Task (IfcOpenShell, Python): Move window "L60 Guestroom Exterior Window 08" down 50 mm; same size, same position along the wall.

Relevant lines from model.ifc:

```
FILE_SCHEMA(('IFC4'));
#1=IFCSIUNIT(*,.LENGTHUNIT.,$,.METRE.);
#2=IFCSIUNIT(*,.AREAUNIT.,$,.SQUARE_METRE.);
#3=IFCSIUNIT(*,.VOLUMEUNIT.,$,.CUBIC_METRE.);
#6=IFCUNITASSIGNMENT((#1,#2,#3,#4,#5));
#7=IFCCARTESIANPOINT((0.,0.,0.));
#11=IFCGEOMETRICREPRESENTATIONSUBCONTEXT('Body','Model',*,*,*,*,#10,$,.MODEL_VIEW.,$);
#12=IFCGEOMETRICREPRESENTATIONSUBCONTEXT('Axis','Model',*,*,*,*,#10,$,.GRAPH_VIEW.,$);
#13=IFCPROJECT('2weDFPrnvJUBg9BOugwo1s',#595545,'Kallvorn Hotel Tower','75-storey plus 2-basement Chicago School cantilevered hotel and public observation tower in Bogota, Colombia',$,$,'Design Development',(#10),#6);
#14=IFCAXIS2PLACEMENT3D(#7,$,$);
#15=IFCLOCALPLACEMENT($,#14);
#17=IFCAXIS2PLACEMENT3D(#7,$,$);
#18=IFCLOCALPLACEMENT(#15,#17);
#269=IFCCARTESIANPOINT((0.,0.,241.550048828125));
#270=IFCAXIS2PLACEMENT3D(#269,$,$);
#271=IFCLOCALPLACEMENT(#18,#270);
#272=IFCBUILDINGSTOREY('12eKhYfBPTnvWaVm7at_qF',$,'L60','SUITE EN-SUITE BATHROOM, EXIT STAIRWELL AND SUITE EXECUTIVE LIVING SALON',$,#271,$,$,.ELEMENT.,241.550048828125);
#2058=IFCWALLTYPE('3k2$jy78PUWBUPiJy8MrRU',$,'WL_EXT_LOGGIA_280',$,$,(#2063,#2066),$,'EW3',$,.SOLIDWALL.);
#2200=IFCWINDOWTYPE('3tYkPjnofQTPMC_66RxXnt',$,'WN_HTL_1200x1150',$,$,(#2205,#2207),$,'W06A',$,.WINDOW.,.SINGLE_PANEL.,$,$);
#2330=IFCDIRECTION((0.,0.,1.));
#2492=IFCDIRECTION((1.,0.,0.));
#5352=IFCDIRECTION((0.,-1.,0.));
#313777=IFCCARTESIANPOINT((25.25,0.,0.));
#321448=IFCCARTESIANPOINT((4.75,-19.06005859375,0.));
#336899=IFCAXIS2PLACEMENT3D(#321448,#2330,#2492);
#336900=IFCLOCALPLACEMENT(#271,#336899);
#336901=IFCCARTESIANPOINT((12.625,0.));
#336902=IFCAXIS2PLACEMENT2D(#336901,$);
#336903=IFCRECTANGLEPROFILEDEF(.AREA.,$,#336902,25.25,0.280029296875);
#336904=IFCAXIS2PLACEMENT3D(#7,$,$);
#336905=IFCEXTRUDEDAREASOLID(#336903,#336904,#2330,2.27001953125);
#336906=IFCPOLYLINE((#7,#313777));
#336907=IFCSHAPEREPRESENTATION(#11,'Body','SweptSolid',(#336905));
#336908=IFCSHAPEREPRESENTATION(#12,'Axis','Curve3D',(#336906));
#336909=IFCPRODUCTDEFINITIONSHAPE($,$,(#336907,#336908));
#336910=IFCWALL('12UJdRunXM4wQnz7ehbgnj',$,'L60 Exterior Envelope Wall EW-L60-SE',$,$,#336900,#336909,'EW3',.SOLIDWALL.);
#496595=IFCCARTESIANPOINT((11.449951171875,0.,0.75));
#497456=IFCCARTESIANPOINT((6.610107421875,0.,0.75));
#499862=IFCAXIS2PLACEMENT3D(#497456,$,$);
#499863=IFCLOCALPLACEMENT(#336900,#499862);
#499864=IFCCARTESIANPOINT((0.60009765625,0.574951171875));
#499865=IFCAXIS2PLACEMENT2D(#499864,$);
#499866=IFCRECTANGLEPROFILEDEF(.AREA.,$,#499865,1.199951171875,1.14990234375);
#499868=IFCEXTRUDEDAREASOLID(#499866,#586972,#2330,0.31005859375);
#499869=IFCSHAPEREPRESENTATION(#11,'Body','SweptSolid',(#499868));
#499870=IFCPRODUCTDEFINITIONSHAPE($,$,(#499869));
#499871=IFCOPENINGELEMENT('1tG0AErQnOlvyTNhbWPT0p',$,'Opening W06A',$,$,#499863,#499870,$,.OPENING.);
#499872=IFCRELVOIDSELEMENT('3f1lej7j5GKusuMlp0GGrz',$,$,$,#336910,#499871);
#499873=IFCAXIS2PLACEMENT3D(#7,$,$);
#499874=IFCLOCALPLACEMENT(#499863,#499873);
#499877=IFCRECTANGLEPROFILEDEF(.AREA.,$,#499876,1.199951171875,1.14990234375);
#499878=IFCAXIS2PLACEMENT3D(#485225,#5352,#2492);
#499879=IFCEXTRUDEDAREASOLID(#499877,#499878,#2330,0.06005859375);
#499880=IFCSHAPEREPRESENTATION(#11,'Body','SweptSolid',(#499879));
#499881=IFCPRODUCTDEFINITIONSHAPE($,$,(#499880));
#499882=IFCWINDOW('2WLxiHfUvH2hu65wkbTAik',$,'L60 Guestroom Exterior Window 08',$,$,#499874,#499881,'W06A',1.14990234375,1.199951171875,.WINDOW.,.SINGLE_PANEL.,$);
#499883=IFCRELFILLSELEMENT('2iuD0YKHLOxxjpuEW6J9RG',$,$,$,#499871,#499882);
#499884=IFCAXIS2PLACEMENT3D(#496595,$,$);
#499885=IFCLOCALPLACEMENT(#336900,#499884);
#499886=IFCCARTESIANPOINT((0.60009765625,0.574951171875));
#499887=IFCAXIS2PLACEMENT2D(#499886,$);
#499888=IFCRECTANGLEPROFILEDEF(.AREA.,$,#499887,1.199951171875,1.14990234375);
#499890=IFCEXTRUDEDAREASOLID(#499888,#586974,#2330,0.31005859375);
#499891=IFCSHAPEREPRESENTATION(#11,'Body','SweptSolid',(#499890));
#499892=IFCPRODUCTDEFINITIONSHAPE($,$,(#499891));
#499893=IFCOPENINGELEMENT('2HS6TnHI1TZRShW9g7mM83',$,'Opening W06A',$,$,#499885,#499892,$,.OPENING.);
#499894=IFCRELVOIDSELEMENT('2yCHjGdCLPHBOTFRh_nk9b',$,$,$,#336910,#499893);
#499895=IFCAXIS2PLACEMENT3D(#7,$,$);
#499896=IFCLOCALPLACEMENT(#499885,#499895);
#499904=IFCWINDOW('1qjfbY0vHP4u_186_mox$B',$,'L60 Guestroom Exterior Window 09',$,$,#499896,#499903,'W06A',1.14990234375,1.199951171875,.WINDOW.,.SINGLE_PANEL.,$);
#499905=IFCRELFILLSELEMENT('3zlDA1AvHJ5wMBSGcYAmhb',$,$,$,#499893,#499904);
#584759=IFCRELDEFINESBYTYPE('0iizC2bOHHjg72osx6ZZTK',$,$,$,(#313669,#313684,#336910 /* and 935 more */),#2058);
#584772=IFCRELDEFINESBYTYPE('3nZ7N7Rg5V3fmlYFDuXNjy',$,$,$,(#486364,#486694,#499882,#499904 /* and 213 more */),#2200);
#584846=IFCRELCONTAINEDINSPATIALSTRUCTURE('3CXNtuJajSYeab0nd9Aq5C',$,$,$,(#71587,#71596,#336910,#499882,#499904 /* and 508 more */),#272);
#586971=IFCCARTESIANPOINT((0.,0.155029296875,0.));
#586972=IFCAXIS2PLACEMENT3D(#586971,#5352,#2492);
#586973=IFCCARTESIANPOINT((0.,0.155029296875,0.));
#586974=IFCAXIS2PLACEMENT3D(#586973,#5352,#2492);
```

```python
import numpy as np
import ifcopenshell
import ifcopenshell.api.geometry
import ifcopenshell.util.placement
import ifcopenshell.util.unit

model = ifcopenshell.open("model.ifc")
unit_scale = ifcopenshell.util.unit.calculate_unit_scale(model)

window = model.by_guid("2WLxiHfUvH2hu65wkbTAik")
opening = window.FillsVoids[0].RelatingOpeningElement
dz = -0.05

shift = np.array([0.0, 0.0, dz])
# The window is placed relative to its opening, so it follows when the opening moves.
matrix = ifcopenshell.util.placement.get_local_placement(opening.ObjectPlacement)
matrix[:3, 3] += shift
ifcopenshell.api.geometry.edit_object_placement(
    model, product=opening, matrix=matrix, is_si=False, should_transform_children=True
)

print(f"moved by {dz * unit_scale:+.3f} m")

model.write("model_v2.ifc")
```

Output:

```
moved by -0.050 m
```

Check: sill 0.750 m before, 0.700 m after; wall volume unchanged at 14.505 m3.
